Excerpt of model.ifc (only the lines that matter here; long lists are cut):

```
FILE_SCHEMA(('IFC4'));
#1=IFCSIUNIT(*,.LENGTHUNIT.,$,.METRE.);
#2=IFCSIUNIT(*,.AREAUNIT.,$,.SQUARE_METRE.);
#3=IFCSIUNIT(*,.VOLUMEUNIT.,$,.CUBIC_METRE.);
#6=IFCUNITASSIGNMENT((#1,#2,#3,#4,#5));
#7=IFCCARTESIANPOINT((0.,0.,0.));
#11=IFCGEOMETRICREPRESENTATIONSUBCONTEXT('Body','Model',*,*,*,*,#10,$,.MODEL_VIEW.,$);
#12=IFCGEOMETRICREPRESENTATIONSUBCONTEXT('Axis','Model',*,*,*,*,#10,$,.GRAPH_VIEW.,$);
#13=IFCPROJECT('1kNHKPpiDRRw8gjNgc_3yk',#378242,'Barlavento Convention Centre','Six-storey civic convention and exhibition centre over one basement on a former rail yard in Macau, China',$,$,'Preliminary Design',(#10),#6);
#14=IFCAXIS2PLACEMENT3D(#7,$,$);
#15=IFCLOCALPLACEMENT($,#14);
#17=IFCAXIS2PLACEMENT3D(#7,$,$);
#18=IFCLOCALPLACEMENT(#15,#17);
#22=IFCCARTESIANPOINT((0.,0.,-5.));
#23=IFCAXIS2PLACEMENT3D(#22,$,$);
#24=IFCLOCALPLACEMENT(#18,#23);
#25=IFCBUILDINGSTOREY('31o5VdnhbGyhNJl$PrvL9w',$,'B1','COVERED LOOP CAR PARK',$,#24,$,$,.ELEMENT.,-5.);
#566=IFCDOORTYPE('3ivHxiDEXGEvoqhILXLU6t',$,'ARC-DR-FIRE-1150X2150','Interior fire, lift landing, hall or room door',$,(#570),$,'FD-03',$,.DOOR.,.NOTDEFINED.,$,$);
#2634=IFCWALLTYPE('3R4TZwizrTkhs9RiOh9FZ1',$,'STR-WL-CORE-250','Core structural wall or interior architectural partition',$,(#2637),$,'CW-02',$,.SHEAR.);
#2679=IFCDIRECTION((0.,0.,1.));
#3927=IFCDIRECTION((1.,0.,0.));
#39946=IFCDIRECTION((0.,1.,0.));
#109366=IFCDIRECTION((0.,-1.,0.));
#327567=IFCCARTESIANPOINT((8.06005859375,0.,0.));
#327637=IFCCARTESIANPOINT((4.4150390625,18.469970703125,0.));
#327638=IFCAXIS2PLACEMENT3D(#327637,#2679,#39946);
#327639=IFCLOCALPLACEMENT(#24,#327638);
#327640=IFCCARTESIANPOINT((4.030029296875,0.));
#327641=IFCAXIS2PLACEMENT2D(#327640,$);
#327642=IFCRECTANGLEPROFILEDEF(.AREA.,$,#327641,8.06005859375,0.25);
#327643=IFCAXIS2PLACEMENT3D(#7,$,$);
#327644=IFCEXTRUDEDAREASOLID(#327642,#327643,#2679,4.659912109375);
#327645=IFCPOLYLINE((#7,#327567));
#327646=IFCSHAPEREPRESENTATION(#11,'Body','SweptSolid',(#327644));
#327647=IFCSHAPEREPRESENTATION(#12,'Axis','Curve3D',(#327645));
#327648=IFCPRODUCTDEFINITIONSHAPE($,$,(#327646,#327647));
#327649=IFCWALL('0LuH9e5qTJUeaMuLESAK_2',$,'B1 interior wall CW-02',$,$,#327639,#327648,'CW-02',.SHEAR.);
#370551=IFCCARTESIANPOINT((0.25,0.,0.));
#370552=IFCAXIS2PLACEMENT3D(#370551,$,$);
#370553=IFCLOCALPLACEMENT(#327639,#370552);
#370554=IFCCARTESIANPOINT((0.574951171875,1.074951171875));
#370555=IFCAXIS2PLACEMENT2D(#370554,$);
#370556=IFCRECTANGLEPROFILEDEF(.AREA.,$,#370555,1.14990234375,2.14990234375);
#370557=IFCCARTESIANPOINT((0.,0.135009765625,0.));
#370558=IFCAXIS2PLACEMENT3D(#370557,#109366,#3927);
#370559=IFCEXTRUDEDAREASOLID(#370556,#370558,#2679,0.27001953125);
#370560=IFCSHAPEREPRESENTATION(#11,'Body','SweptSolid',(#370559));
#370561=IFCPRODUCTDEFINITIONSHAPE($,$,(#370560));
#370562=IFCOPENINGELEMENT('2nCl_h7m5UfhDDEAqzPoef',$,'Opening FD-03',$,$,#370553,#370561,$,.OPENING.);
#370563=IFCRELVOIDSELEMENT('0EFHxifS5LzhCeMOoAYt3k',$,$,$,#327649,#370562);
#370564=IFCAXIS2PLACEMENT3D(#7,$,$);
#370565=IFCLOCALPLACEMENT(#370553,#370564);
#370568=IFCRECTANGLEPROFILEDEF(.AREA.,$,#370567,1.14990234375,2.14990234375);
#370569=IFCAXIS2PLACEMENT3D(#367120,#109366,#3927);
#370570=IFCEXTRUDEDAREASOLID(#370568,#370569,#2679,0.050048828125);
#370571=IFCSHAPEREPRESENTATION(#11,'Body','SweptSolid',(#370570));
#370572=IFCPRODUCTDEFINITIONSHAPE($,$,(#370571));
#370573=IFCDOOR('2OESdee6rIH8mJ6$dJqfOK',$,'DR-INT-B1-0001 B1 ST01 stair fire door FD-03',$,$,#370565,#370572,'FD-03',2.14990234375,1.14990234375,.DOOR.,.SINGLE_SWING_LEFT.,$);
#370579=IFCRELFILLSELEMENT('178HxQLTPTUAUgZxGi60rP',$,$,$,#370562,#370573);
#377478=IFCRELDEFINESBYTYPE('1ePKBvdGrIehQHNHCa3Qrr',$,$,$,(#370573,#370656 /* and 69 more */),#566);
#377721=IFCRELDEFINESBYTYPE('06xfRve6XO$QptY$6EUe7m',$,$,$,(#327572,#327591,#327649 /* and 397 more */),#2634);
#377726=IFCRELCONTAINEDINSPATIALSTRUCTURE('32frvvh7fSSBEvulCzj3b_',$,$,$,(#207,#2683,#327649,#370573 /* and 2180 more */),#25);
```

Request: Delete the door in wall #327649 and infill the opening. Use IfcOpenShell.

```python
import ifcopenshell
import ifcopenshell.api.feature
import ifcopenshell.api.root
import ifcopenshell.geom
import ifcopenshell.util.shape

model = ifcopenshell.open("model.ifc")
settings = ifcopenshell.geom.settings()


def volume(element):
    """Net volume in cubic metres, openings subtracted."""
    shape = ifcopenshell.geom.create_shape(settings, element)
    return ifcopenshell.util.shape.get_volume(shape.geometry)


door = model.by_guid("2OESdee6rIH8mJ6$dJqfOK")
opening = door.FillsVoids[0].RelatingOpeningElement
wall = opening.VoidsElements[0].RelatingBuildingElement
before = volume(wall)

ifcopenshell.api.root.remove_product(model, product=door)
ifcopenshell.api.feature.remove_feature(model, feature=opening)

after = volume(wall)

print(f"wall volume {before:.3f} -> {after:.3f} m3")

model.write("model_edited.ifc")
```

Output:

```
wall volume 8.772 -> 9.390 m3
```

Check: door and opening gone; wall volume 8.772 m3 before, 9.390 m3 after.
